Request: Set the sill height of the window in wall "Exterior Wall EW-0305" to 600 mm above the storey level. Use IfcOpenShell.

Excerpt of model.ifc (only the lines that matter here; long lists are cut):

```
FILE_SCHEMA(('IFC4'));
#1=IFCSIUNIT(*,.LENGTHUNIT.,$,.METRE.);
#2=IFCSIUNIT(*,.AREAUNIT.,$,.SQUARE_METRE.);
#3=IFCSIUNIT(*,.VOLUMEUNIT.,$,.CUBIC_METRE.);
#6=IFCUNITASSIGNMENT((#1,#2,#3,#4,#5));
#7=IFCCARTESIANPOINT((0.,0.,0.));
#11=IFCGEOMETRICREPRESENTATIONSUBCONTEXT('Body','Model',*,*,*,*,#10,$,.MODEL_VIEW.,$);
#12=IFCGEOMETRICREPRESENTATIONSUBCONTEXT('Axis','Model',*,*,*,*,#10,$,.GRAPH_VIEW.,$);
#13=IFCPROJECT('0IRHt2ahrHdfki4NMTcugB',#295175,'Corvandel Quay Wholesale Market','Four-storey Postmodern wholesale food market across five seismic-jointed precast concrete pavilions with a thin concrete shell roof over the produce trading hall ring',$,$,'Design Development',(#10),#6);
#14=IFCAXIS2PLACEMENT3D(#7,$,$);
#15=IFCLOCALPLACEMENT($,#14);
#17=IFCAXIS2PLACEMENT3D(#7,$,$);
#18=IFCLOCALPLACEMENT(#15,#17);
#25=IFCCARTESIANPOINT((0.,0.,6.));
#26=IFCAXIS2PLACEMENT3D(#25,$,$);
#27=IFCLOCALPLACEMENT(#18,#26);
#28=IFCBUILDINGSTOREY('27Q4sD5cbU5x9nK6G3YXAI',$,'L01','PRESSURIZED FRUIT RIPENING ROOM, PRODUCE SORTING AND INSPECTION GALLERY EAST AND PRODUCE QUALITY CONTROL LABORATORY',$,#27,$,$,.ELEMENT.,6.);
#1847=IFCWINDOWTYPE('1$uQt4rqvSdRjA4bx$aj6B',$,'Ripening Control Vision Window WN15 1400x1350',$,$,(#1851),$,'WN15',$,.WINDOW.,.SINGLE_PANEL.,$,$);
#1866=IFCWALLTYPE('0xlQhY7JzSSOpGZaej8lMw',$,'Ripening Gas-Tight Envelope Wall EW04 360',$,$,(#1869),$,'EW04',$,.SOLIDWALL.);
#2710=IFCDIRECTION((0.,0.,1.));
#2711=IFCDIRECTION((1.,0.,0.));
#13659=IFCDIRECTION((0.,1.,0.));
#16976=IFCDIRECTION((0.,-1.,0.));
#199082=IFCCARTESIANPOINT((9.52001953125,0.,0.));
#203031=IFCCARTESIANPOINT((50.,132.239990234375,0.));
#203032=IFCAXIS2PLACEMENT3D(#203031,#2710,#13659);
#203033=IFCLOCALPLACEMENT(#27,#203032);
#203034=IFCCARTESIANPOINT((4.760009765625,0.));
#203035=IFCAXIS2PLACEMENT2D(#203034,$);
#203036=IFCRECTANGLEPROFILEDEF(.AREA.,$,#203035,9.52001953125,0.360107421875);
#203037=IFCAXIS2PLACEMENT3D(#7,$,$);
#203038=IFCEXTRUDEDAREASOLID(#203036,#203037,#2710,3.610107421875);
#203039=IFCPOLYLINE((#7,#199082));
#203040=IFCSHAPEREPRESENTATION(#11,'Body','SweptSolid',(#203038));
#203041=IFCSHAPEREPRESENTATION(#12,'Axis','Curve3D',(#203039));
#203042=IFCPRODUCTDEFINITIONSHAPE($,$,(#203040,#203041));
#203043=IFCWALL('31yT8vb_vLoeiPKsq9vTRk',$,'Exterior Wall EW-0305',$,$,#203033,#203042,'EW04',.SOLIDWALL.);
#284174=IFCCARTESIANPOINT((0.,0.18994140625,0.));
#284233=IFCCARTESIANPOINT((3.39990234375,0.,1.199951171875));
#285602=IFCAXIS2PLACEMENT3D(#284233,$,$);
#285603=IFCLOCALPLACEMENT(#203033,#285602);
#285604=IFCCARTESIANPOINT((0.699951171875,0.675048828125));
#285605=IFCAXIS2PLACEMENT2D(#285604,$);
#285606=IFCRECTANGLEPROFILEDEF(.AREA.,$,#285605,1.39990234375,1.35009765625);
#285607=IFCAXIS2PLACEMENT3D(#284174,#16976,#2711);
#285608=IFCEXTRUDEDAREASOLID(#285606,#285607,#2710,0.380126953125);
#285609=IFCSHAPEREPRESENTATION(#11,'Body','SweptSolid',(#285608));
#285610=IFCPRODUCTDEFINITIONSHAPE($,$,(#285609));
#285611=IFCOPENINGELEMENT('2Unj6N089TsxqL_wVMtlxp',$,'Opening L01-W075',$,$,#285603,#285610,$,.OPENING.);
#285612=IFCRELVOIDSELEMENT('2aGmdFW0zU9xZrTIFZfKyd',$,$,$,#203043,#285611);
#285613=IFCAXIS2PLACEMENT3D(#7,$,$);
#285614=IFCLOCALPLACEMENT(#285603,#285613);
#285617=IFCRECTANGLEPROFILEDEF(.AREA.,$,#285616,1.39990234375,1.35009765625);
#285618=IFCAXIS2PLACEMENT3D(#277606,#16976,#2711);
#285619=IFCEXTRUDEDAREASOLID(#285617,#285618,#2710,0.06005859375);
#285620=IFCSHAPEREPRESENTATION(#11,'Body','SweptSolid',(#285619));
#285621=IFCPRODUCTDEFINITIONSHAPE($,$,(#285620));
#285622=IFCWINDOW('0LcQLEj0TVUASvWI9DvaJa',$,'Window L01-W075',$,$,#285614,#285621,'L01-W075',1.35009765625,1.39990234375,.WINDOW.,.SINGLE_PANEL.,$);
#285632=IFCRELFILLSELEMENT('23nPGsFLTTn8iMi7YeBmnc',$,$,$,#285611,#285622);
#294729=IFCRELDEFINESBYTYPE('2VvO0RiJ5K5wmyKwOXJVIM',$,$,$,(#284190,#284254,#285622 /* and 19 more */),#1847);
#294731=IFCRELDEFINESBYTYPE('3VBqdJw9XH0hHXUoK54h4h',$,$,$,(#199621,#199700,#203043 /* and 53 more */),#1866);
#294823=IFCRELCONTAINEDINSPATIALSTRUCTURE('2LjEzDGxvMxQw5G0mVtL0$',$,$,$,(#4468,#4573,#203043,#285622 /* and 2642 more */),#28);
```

```python
import numpy as np
import ifcopenshell
import ifcopenshell.api.geometry
import ifcopenshell.geom
import ifcopenshell.util.element
import ifcopenshell.util.placement
import ifcopenshell.util.shape
import ifcopenshell.util.unit

model = ifcopenshell.open("model.ifc")
unit_scale = ifcopenshell.util.unit.calculate_unit_scale(model)

window = model.by_guid("0LcQLEj0TVUASvWI9DvaJa")
opening = window.FillsVoids[0].RelatingOpeningElement
storey = ifcopenshell.util.element.get_container(window, ifc_class="IfcBuildingStorey")
level = ifcopenshell.util.placement.get_local_placement(storey.ObjectPlacement)[2, 3]

# The opening's origin need not be at the sill, so measure its lowest point.
shape = ifcopenshell.geom.create_shape(ifcopenshell.geom.settings(), opening)
bottom = ifcopenshell.util.shape.get_shape_bottom_elevation(shape, shape.geometry) / unit_scale
dz = level + 0.6 / unit_scale - bottom

shift = np.array([0.0, 0.0, dz])
# The window is placed relative to its opening, so it follows when the opening moves.
matrix = ifcopenshell.util.placement.get_local_placement(opening.ObjectPlacement)
matrix[:3, 3] += shift
ifcopenshell.api.geometry.edit_object_placement(
    model, product=opening, matrix=matrix, is_si=False, should_transform_children=True
)

print(f"moved by {dz * unit_scale:+.3f} m")

model.write("model_updated.ifc")
```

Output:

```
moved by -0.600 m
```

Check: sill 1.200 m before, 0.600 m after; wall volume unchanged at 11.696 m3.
